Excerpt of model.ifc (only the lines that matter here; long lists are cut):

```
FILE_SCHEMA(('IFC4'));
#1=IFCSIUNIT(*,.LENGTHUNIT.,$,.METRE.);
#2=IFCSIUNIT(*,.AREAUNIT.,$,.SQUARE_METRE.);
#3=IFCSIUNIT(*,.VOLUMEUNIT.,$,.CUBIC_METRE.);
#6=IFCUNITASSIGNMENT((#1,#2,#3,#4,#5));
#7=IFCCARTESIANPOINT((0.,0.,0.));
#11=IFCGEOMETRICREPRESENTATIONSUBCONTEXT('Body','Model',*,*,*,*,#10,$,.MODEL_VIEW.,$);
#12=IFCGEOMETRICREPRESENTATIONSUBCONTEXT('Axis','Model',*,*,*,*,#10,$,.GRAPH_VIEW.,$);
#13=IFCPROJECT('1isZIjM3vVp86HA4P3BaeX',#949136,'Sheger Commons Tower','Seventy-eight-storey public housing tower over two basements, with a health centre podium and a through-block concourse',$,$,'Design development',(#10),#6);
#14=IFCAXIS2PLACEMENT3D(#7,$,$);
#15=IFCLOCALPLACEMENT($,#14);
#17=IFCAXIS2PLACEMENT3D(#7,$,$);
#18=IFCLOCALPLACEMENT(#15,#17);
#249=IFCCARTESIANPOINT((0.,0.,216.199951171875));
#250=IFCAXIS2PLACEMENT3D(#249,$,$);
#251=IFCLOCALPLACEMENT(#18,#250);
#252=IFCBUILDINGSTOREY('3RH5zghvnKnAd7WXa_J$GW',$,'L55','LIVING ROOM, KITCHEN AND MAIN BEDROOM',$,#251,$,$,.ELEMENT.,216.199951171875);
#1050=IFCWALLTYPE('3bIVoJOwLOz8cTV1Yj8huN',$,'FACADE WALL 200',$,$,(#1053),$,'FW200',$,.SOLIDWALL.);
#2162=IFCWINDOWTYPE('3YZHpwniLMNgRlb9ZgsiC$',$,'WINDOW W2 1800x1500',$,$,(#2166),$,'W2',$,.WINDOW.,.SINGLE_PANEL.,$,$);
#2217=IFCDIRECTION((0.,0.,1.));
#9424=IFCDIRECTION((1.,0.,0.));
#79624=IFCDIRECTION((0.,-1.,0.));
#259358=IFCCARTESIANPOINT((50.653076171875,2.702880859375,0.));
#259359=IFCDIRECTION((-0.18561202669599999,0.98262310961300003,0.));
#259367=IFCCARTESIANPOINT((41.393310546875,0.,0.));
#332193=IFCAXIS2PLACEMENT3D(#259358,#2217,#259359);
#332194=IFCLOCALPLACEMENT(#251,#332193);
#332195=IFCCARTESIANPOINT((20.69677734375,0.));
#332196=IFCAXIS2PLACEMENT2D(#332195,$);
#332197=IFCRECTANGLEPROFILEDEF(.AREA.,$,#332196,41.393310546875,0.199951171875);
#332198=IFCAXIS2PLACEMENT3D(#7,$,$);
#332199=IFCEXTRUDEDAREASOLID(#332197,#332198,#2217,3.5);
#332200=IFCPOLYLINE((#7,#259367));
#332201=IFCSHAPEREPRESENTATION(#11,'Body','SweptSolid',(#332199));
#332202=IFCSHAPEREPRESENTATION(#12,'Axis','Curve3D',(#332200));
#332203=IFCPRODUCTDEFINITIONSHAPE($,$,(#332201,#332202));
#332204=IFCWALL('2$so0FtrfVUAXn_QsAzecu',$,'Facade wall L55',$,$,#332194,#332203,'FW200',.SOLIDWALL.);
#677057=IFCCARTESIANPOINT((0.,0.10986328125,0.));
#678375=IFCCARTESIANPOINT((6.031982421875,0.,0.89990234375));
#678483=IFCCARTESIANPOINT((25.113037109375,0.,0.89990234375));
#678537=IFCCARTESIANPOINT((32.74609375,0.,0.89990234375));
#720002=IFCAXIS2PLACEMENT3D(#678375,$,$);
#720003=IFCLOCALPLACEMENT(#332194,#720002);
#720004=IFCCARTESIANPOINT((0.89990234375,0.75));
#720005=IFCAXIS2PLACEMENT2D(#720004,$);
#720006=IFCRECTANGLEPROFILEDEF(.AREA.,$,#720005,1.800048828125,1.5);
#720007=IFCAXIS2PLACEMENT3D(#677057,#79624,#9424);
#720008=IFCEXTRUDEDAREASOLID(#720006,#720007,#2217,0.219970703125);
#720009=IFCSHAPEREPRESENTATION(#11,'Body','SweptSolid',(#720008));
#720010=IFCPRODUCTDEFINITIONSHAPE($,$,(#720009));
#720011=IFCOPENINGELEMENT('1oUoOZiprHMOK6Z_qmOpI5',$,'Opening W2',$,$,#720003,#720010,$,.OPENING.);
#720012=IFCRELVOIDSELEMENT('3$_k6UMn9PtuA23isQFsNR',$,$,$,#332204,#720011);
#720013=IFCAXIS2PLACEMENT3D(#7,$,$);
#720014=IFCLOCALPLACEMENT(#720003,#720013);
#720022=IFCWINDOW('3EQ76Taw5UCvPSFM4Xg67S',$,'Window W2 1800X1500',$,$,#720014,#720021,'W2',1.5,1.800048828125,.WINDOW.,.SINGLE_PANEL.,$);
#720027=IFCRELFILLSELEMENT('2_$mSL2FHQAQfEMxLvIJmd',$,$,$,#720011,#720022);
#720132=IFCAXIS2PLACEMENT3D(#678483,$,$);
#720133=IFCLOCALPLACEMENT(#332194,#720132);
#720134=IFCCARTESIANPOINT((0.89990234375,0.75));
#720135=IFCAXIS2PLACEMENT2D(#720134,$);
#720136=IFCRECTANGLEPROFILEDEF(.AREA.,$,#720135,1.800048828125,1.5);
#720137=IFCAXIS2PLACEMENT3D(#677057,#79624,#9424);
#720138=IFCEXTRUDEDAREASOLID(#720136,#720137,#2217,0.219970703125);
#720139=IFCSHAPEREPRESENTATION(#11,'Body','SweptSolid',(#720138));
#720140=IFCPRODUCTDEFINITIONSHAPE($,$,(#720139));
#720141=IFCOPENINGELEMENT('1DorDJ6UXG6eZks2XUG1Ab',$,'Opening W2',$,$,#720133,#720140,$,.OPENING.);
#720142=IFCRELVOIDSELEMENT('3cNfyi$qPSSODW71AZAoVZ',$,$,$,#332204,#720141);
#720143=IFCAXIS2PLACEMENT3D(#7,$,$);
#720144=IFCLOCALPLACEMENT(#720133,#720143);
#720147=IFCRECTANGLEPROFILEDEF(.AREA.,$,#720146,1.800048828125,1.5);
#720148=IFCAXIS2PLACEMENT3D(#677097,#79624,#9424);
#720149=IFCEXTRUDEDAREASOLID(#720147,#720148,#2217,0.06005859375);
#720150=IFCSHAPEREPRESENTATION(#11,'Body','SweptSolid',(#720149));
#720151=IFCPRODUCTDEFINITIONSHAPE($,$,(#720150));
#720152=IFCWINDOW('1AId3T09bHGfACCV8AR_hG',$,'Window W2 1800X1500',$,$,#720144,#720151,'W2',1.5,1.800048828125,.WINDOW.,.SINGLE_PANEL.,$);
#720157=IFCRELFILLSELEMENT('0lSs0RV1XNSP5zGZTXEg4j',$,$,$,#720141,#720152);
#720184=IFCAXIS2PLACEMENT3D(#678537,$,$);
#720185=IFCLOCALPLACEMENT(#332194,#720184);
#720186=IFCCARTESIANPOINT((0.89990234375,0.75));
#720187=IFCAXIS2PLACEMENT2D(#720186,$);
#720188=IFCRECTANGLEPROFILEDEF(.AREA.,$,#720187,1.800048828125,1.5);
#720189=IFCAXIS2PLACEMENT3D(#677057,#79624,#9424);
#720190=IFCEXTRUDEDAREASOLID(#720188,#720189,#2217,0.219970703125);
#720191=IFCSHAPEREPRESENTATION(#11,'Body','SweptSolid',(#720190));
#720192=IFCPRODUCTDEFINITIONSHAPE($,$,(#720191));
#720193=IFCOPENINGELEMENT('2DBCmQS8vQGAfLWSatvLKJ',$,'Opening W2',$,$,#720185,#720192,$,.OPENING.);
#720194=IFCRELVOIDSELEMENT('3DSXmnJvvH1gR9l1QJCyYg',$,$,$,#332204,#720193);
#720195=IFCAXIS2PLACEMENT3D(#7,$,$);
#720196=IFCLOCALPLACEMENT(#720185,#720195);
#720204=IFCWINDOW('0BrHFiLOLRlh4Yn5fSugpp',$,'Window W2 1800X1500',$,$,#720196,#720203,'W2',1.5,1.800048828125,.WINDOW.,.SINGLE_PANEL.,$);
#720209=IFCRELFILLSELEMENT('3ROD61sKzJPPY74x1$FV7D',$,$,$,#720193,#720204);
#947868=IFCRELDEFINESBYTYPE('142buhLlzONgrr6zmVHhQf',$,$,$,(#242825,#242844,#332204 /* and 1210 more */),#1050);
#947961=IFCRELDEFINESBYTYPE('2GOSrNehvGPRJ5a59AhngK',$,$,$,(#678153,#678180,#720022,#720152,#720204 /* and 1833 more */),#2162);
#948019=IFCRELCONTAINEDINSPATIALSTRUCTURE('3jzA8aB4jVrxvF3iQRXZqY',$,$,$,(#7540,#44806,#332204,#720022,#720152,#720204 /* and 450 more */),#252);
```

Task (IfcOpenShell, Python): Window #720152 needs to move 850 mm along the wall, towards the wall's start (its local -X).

```python
import ifcopenshell
import ifcopenshell.api.geometry
import ifcopenshell.util.placement
import ifcopenshell.util.unit

model = ifcopenshell.open("model.ifc")
unit_scale = ifcopenshell.util.unit.calculate_unit_scale(model)

window = model.by_guid("1AId3T09bHGfACCV8AR_hG")
opening = window.FillsVoids[0].RelatingOpeningElement
wall = opening.VoidsElements[0].RelatingBuildingElement

wall_matrix = ifcopenshell.util.placement.get_local_placement(wall.ObjectPlacement)
shift = wall_matrix[:3, 0] * -0.85 / unit_scale
before = ifcopenshell.util.placement.get_local_placement(window.ObjectPlacement)[:3, 3].copy()

# The window is placed relative to its opening, so it follows when the opening moves.
matrix = ifcopenshell.util.placement.get_local_placement(opening.ObjectPlacement)
matrix[:3, 3] += shift
ifcopenshell.api.geometry.edit_object_placement(
    model, product=opening, matrix=matrix, is_si=False, should_transform_children=True
)

after = ifcopenshell.util.placement.get_local_placement(window.ObjectPlacement)[:3, 3]
print("window moved by", (after - before).round(3) + 0.0)

model.write("model_v2.ifc")
```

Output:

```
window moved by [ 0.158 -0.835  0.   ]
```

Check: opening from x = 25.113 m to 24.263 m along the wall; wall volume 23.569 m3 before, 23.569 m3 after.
